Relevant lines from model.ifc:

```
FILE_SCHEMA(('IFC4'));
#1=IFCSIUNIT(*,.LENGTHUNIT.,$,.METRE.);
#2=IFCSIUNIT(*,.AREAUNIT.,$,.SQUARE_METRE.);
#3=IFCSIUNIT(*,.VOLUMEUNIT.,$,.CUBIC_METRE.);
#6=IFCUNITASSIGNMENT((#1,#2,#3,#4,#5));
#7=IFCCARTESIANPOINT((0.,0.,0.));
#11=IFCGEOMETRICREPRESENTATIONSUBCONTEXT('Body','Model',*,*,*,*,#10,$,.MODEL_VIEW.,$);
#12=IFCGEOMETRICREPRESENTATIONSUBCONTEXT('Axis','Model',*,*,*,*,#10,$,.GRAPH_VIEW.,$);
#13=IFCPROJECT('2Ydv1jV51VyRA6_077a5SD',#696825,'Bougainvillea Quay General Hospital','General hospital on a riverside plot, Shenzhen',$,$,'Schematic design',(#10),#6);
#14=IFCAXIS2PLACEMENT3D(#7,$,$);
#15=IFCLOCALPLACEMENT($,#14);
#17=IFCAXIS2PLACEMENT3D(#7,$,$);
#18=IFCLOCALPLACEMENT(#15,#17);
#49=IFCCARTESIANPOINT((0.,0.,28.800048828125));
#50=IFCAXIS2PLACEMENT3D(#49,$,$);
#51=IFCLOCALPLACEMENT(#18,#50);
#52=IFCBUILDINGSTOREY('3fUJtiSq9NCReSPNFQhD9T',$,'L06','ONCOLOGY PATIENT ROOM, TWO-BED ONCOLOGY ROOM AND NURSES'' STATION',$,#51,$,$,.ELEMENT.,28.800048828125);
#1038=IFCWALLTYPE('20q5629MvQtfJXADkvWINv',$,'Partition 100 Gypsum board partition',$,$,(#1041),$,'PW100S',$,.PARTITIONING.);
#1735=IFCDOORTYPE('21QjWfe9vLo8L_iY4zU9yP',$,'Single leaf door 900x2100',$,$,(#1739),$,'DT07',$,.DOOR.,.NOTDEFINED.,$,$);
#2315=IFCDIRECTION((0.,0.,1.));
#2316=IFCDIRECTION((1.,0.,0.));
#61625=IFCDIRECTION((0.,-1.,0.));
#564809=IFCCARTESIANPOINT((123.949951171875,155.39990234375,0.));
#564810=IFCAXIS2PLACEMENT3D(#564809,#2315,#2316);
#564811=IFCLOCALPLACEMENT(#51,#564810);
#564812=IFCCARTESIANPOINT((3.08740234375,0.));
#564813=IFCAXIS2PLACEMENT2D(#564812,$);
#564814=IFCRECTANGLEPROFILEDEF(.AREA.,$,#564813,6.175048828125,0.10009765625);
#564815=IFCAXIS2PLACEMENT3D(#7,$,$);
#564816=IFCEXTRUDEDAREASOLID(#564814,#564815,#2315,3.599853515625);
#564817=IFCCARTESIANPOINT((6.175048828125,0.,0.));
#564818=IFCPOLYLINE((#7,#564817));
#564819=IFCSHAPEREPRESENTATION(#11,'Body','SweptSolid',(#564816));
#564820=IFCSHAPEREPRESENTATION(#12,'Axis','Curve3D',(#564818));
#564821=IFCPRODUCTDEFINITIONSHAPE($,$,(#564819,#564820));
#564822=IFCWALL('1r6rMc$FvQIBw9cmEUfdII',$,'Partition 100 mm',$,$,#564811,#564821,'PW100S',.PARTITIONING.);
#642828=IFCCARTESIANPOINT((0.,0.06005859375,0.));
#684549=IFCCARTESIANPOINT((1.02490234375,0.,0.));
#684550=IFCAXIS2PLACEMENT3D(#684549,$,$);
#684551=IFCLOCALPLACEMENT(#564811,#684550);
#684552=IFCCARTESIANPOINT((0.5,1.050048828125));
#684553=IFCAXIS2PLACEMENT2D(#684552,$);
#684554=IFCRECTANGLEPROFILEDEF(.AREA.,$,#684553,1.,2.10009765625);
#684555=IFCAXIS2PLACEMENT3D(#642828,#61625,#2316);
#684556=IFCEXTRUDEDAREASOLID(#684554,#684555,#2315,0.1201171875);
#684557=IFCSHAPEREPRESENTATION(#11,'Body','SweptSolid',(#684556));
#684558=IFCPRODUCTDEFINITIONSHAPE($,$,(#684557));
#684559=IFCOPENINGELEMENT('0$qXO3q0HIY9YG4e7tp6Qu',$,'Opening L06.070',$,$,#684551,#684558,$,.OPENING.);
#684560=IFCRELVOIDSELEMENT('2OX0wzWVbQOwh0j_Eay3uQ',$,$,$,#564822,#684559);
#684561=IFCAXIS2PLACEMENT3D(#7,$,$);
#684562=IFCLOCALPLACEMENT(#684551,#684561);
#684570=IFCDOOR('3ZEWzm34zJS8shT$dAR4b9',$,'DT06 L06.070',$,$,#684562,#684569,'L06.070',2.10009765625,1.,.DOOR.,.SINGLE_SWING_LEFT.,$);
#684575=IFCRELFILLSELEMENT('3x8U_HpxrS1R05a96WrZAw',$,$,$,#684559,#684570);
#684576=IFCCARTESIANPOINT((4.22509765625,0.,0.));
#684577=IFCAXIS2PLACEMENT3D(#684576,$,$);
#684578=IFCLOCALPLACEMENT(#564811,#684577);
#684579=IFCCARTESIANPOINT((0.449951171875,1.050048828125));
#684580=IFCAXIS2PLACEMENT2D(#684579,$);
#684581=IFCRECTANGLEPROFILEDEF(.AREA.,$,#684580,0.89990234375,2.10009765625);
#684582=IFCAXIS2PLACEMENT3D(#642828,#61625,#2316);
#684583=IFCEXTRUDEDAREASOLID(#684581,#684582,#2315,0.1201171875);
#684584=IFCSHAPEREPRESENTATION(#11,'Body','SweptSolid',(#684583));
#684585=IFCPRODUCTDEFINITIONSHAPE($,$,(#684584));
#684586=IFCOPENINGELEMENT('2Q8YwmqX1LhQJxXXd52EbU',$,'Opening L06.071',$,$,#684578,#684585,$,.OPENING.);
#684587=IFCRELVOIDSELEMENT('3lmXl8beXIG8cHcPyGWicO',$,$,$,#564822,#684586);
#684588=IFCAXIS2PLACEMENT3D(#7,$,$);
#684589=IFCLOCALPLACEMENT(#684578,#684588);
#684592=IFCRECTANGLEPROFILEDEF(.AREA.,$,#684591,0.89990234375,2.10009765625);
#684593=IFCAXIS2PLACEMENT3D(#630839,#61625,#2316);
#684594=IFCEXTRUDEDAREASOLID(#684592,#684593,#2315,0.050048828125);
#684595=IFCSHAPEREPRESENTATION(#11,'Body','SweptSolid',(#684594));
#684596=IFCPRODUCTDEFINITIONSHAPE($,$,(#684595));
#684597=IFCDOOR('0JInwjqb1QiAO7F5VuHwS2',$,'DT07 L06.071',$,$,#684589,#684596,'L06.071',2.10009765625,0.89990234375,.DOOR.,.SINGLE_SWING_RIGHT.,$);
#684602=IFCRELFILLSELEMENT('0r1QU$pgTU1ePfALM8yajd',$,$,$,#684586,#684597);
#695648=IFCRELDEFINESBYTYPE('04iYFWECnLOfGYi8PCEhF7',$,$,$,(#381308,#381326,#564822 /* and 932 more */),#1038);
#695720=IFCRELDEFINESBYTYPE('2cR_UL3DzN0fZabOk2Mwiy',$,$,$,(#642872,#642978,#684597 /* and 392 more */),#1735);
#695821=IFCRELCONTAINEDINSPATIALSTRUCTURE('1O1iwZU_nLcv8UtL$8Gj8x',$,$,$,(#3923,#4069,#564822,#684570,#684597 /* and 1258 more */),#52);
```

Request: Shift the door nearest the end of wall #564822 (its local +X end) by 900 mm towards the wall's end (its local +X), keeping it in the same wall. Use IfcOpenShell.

```python
import ifcopenshell
import ifcopenshell.api.geometry
import ifcopenshell.util.placement
import ifcopenshell.util.unit

model = ifcopenshell.open("model.ifc")
unit_scale = ifcopenshell.util.unit.calculate_unit_scale(model)

door = model.by_guid("0JInwjqb1QiAO7F5VuHwS2")
opening = door.FillsVoids[0].RelatingOpeningElement
wall = opening.VoidsElements[0].RelatingBuildingElement

wall_matrix = ifcopenshell.util.placement.get_local_placement(wall.ObjectPlacement)
shift = wall_matrix[:3, 0] * 0.9 / unit_scale
before = ifcopenshell.util.placement.get_local_placement(door.ObjectPlacement)[:3, 3].copy()

# The door is placed relative to its opening, so it follows when the opening moves.
matrix = ifcopenshell.util.placement.get_local_placement(opening.ObjectPlacement)
matrix[:3, 3] += shift
ifcopenshell.api.geometry.edit_object_placement(
    model, product=opening, matrix=matrix, is_si=False, should_transform_children=True
)

after = ifcopenshell.util.placement.get_local_placement(door.ObjectPlacement)[:3, 3]
print("door moved by", (after - before).round(3) + 0.0)

model.write("model_updated.ifc")
```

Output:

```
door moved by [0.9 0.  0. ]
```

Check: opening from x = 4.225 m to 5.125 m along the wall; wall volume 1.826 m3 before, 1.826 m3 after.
